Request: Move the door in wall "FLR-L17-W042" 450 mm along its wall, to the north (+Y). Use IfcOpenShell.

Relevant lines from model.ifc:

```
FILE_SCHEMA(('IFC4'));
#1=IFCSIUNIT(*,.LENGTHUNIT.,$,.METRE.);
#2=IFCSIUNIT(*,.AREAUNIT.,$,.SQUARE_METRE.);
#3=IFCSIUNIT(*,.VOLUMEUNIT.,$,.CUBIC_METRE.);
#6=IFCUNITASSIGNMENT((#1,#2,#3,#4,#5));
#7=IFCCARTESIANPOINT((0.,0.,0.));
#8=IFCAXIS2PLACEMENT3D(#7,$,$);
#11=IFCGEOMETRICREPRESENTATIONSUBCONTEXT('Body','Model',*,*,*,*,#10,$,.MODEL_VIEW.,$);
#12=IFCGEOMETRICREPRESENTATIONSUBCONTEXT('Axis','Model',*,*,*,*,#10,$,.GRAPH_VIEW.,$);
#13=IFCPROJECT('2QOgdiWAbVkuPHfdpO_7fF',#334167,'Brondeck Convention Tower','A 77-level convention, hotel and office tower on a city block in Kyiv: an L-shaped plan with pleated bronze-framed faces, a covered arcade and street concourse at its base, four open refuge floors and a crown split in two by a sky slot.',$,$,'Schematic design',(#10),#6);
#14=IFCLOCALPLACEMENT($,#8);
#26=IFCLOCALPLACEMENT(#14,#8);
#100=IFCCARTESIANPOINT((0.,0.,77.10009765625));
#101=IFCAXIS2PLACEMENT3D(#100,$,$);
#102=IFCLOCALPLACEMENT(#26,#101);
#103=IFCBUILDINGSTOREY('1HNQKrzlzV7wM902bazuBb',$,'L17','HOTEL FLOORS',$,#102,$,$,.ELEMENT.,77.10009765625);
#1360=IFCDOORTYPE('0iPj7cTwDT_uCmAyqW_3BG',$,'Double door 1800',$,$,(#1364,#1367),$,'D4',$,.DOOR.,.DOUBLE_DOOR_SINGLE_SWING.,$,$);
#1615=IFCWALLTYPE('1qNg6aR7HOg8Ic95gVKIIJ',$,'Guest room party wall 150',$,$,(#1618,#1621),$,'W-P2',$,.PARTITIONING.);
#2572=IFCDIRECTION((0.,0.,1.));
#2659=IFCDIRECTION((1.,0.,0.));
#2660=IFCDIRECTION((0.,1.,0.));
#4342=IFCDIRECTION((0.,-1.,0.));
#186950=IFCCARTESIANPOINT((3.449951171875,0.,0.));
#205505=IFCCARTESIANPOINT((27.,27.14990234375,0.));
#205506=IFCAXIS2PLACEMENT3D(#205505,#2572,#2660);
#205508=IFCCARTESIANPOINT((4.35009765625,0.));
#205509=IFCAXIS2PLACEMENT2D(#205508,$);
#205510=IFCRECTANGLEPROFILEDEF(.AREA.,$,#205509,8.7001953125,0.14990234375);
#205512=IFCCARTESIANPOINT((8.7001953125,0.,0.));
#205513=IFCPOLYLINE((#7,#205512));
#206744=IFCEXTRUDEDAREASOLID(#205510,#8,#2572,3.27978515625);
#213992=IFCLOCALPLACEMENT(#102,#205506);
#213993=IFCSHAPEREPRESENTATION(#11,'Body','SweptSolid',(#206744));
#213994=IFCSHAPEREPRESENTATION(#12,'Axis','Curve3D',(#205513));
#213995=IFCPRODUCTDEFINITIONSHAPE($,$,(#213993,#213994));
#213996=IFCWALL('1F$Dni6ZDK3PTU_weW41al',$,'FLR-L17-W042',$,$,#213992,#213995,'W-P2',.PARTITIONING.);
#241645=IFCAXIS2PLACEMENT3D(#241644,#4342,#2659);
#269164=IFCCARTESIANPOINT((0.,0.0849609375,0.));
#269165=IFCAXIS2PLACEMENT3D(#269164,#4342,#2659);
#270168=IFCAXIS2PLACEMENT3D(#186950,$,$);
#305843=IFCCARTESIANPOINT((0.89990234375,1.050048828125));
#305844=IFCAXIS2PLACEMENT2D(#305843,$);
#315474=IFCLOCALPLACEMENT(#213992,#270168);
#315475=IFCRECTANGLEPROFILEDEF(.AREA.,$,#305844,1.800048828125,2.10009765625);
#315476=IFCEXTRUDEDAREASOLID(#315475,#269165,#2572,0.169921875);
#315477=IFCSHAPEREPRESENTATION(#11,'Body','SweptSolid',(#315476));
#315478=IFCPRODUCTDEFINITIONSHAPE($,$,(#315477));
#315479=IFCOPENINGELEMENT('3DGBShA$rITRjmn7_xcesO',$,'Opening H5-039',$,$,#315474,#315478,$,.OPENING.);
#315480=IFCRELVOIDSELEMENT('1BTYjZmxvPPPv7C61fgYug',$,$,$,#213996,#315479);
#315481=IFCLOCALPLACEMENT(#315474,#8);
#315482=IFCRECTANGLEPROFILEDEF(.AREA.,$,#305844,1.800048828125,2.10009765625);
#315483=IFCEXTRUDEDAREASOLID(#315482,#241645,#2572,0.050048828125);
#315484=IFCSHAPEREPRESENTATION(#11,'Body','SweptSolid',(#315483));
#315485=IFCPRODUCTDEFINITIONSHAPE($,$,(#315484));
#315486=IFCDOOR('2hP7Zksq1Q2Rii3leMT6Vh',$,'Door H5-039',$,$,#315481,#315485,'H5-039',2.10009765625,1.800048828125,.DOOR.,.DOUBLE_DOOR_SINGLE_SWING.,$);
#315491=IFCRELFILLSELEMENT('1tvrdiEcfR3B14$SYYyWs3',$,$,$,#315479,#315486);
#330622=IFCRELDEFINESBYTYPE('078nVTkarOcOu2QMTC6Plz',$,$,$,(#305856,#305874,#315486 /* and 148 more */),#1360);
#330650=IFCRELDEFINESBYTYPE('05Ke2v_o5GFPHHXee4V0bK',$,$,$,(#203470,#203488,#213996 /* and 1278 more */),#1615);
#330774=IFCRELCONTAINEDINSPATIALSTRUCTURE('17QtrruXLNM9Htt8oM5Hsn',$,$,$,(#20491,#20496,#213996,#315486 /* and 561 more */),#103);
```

```python
import ifcopenshell
import ifcopenshell.api.geometry
import ifcopenshell.util.placement
import ifcopenshell.util.unit

model = ifcopenshell.open("model.ifc")
unit_scale = ifcopenshell.util.unit.calculate_unit_scale(model)

door = model.by_guid("2hP7Zksq1Q2Rii3leMT6Vh")
opening = door.FillsVoids[0].RelatingOpeningElement
wall = opening.VoidsElements[0].RelatingBuildingElement

wall_matrix = ifcopenshell.util.placement.get_local_placement(wall.ObjectPlacement)
shift = wall_matrix[:3, 0] * 0.45 / unit_scale
before = ifcopenshell.util.placement.get_local_placement(door.ObjectPlacement)[:3, 3].copy()

# The door is placed relative to its opening, so it follows when the opening moves.
matrix = ifcopenshell.util.placement.get_local_placement(opening.ObjectPlacement)
matrix[:3, 3] += shift
ifcopenshell.api.geometry.edit_object_placement(
    model, product=opening, matrix=matrix, is_si=False, should_transform_children=True
)

after = ifcopenshell.util.placement.get_local_placement(door.ObjectPlacement)[:3, 3]
print("door moved by", (after - before).round(3) + 0.0)

model.write("model-out.ifc")
```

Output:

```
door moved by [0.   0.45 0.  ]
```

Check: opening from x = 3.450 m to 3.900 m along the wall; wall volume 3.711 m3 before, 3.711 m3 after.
